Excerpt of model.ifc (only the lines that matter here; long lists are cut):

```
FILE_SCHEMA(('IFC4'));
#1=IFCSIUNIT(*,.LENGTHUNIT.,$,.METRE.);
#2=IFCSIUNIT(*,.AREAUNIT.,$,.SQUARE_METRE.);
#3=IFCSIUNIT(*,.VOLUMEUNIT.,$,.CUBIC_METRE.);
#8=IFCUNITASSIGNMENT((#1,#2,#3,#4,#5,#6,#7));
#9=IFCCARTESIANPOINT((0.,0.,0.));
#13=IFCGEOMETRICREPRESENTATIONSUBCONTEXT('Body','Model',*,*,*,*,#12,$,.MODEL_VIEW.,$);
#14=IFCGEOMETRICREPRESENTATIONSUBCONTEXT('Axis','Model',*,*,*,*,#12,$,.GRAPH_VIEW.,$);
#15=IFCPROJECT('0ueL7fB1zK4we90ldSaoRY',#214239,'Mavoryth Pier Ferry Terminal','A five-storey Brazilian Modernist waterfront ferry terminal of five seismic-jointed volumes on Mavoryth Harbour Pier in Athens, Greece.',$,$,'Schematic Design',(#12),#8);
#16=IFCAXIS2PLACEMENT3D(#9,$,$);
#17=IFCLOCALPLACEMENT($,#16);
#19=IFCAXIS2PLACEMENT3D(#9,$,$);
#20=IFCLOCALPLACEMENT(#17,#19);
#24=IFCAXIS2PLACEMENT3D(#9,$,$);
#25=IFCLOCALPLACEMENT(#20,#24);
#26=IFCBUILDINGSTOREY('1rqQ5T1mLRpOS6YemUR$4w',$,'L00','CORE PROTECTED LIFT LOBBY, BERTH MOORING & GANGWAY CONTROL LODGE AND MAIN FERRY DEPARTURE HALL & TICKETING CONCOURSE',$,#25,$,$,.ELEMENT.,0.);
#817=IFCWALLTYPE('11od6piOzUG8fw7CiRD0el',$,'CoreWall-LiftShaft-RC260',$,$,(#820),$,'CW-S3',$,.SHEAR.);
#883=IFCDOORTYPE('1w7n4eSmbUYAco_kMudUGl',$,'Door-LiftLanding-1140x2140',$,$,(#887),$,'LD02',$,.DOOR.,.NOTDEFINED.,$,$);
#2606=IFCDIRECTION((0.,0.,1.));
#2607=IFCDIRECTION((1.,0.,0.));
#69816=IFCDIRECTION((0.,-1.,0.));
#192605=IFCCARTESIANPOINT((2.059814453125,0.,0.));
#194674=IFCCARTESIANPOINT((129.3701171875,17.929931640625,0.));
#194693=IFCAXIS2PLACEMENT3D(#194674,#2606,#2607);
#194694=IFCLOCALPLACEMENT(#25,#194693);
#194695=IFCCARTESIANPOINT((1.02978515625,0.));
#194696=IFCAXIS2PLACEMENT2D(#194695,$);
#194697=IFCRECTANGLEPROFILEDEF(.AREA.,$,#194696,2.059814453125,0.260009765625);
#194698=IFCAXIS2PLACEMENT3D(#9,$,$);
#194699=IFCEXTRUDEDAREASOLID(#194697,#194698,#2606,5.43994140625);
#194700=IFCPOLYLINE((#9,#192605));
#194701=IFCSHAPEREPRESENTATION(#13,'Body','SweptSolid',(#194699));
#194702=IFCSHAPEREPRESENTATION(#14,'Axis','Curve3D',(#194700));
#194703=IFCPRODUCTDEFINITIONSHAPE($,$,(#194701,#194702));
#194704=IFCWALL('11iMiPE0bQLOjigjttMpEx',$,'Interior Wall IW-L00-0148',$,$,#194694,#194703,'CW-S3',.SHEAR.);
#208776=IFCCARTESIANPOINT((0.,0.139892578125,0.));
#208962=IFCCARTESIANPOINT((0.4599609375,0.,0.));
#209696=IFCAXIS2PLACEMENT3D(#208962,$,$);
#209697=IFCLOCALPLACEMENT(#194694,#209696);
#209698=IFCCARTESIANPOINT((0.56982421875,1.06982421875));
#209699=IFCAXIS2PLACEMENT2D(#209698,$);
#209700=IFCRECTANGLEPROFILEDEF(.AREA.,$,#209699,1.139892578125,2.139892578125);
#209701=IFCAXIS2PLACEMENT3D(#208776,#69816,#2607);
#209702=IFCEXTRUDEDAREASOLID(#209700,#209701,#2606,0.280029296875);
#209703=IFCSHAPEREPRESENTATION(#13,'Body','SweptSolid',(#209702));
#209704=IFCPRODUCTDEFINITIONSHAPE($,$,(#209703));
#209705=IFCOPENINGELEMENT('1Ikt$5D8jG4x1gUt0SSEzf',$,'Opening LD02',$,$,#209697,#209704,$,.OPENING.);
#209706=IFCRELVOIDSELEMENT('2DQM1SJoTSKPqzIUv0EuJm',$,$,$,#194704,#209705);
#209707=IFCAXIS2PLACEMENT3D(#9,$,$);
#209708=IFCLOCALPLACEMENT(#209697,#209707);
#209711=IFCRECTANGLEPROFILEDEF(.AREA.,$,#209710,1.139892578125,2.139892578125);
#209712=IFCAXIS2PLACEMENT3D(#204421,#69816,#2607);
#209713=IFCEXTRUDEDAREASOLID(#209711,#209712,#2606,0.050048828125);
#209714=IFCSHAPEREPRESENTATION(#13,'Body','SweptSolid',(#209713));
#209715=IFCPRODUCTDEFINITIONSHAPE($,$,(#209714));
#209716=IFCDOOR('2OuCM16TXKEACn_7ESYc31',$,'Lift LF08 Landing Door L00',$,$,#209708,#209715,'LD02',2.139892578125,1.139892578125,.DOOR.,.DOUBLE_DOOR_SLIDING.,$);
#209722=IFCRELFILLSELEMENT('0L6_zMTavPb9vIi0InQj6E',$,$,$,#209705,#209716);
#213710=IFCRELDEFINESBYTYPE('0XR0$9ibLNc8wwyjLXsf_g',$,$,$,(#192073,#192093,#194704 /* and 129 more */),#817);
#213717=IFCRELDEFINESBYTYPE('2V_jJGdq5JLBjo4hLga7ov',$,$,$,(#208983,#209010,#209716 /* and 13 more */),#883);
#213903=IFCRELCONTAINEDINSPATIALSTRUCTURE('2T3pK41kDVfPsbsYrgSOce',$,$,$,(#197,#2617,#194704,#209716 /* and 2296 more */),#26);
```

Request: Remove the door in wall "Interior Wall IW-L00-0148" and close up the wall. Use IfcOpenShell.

```python
import ifcopenshell
import ifcopenshell.api.feature
import ifcopenshell.api.root
import ifcopenshell.geom
import ifcopenshell.util.shape

model = ifcopenshell.open("model.ifc")
settings = ifcopenshell.geom.settings()


def volume(element):
    """Net volume in cubic metres, openings subtracted."""
    shape = ifcopenshell.geom.create_shape(settings, element)
    return ifcopenshell.util.shape.get_volume(shape.geometry)


door = model.by_guid("2OuCM16TXKEACn_7ESYc31")
opening = door.FillsVoids[0].RelatingOpeningElement
wall = opening.VoidsElements[0].RelatingBuildingElement
before = volume(wall)

ifcopenshell.api.root.remove_product(model, product=door)
ifcopenshell.api.feature.remove_feature(model, feature=opening)

after = volume(wall)

print(f"wall volume {before:.3f} -> {after:.3f} m3")

model.write("model_rev.ifc")
```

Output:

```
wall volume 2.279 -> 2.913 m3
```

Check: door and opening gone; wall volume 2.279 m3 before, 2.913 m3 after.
